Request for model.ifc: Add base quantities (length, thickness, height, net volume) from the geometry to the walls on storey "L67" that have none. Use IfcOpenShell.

First a look at what the model holds.

```python
import ifcopenshell
import ifcopenshell.util.element
import ifcopenshell.util.unit

model = ifcopenshell.open("model.ifc")
print(model.schema)
for unit_type in ("LENGTHUNIT", "AREAUNIT", "VOLUMEUNIT"):
    print(unit_type, ifcopenshell.util.unit.calculate_unit_scale(model, unit_type))
storey = next(s for s in model.by_type("IfcBuildingStorey") if s.Name == "L67")
walls = [e for e in ifcopenshell.util.element.get_decomposition(storey) if e.is_a("IfcWall")]
for e in sorted(walls, key=lambda e: e.id()):
    print(e.id(), e.is_a(), e.Name, list(ifcopenshell.util.element.get_psets(e, qtos_only=True)), sep=" | ")
```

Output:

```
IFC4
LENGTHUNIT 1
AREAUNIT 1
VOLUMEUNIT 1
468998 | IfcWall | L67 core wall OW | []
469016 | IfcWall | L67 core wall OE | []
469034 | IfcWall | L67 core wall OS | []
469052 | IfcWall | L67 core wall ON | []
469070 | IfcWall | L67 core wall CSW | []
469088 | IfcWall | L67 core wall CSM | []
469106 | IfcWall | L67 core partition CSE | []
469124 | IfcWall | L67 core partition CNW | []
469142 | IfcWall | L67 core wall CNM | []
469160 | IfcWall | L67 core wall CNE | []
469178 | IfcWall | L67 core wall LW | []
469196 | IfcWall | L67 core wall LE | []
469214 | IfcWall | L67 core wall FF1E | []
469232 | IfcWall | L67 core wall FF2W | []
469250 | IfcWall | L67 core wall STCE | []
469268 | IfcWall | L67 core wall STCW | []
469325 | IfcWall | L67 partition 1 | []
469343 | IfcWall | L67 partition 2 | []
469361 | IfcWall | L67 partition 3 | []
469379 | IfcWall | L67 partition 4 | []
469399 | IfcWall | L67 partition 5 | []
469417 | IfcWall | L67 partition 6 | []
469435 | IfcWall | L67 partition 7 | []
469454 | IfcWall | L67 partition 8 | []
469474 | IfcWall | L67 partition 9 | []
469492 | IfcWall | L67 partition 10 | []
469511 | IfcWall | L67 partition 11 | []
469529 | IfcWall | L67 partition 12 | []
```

```python
import ifcopenshell
import ifcopenshell.api.pset
import ifcopenshell.geom
import ifcopenshell.util.element
import ifcopenshell.util.shape
import ifcopenshell.util.unit

model = ifcopenshell.open("model.ifc")
unit_scale = ifcopenshell.util.unit.calculate_unit_scale(model)
volume_scale = ifcopenshell.util.unit.calculate_unit_scale(model, "VOLUMEUNIT")
settings = ifcopenshell.geom.settings()

storey = next(s for s in model.by_type("IfcBuildingStorey") if s.Name == "L67")
walls = [e for e in ifcopenshell.util.element.get_decomposition(storey) if e.is_a("IfcWall")]

for e in sorted(walls, key=lambda e: e.id()):
    if ifcopenshell.util.element.get_psets(e, qtos_only=True, should_inherit=False):
        continue
    # Geometry comes back in metres, in the element's own axes.
    shape = ifcopenshell.geom.create_shape(settings, e)
    values = {
        "Length": ifcopenshell.util.shape.get_x(shape.geometry) / unit_scale,
        "Width": ifcopenshell.util.shape.get_y(shape.geometry) / unit_scale,
        "Height": ifcopenshell.util.shape.get_z(shape.geometry) / unit_scale,
        "NetVolume": ifcopenshell.util.shape.get_volume(shape.geometry) / volume_scale,
    }
    qto = ifcopenshell.api.pset.add_qto(model, product=e, name="Qto_WallBaseQuantities")
    ifcopenshell.api.pset.edit_qto(model, qto=qto, properties=values)
    print(e.id(), {k: round(v, 3) for k, v in values.items()})

model.write("model_updated.ifc")
```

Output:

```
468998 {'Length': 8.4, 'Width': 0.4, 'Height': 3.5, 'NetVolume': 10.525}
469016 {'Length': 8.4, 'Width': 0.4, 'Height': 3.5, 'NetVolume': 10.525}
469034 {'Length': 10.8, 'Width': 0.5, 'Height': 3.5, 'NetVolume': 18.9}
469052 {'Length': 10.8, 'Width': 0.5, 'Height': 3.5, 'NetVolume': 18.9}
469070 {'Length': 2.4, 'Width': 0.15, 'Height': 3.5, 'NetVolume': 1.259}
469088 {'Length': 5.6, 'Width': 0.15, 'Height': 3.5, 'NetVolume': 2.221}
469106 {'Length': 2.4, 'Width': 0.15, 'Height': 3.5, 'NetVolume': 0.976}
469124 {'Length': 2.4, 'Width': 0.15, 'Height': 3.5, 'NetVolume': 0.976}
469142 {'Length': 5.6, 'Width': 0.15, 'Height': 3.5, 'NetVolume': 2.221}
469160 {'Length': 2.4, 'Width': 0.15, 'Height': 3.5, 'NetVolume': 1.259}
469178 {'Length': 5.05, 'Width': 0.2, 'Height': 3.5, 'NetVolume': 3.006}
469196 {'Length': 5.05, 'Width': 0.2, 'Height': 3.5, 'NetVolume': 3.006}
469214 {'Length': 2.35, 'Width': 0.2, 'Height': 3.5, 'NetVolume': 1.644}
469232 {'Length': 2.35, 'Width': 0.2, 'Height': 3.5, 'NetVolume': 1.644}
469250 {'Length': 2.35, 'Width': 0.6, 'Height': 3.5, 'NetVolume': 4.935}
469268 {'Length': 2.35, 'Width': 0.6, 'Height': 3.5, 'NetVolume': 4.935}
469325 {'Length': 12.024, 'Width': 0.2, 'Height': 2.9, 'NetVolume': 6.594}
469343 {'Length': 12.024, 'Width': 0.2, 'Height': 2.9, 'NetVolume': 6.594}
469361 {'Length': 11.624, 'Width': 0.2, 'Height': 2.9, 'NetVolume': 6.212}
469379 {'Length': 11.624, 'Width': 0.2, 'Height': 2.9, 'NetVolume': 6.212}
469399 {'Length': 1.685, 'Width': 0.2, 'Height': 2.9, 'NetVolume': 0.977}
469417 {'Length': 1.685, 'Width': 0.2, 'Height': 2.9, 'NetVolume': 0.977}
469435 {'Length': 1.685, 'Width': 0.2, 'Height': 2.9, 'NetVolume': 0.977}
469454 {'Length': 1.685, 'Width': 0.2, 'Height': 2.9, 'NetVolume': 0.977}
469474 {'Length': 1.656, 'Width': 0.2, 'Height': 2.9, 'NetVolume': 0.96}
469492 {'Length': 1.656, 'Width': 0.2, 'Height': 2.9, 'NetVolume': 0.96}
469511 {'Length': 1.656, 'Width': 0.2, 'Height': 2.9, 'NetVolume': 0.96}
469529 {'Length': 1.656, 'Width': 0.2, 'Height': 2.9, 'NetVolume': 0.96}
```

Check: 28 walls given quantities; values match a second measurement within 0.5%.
